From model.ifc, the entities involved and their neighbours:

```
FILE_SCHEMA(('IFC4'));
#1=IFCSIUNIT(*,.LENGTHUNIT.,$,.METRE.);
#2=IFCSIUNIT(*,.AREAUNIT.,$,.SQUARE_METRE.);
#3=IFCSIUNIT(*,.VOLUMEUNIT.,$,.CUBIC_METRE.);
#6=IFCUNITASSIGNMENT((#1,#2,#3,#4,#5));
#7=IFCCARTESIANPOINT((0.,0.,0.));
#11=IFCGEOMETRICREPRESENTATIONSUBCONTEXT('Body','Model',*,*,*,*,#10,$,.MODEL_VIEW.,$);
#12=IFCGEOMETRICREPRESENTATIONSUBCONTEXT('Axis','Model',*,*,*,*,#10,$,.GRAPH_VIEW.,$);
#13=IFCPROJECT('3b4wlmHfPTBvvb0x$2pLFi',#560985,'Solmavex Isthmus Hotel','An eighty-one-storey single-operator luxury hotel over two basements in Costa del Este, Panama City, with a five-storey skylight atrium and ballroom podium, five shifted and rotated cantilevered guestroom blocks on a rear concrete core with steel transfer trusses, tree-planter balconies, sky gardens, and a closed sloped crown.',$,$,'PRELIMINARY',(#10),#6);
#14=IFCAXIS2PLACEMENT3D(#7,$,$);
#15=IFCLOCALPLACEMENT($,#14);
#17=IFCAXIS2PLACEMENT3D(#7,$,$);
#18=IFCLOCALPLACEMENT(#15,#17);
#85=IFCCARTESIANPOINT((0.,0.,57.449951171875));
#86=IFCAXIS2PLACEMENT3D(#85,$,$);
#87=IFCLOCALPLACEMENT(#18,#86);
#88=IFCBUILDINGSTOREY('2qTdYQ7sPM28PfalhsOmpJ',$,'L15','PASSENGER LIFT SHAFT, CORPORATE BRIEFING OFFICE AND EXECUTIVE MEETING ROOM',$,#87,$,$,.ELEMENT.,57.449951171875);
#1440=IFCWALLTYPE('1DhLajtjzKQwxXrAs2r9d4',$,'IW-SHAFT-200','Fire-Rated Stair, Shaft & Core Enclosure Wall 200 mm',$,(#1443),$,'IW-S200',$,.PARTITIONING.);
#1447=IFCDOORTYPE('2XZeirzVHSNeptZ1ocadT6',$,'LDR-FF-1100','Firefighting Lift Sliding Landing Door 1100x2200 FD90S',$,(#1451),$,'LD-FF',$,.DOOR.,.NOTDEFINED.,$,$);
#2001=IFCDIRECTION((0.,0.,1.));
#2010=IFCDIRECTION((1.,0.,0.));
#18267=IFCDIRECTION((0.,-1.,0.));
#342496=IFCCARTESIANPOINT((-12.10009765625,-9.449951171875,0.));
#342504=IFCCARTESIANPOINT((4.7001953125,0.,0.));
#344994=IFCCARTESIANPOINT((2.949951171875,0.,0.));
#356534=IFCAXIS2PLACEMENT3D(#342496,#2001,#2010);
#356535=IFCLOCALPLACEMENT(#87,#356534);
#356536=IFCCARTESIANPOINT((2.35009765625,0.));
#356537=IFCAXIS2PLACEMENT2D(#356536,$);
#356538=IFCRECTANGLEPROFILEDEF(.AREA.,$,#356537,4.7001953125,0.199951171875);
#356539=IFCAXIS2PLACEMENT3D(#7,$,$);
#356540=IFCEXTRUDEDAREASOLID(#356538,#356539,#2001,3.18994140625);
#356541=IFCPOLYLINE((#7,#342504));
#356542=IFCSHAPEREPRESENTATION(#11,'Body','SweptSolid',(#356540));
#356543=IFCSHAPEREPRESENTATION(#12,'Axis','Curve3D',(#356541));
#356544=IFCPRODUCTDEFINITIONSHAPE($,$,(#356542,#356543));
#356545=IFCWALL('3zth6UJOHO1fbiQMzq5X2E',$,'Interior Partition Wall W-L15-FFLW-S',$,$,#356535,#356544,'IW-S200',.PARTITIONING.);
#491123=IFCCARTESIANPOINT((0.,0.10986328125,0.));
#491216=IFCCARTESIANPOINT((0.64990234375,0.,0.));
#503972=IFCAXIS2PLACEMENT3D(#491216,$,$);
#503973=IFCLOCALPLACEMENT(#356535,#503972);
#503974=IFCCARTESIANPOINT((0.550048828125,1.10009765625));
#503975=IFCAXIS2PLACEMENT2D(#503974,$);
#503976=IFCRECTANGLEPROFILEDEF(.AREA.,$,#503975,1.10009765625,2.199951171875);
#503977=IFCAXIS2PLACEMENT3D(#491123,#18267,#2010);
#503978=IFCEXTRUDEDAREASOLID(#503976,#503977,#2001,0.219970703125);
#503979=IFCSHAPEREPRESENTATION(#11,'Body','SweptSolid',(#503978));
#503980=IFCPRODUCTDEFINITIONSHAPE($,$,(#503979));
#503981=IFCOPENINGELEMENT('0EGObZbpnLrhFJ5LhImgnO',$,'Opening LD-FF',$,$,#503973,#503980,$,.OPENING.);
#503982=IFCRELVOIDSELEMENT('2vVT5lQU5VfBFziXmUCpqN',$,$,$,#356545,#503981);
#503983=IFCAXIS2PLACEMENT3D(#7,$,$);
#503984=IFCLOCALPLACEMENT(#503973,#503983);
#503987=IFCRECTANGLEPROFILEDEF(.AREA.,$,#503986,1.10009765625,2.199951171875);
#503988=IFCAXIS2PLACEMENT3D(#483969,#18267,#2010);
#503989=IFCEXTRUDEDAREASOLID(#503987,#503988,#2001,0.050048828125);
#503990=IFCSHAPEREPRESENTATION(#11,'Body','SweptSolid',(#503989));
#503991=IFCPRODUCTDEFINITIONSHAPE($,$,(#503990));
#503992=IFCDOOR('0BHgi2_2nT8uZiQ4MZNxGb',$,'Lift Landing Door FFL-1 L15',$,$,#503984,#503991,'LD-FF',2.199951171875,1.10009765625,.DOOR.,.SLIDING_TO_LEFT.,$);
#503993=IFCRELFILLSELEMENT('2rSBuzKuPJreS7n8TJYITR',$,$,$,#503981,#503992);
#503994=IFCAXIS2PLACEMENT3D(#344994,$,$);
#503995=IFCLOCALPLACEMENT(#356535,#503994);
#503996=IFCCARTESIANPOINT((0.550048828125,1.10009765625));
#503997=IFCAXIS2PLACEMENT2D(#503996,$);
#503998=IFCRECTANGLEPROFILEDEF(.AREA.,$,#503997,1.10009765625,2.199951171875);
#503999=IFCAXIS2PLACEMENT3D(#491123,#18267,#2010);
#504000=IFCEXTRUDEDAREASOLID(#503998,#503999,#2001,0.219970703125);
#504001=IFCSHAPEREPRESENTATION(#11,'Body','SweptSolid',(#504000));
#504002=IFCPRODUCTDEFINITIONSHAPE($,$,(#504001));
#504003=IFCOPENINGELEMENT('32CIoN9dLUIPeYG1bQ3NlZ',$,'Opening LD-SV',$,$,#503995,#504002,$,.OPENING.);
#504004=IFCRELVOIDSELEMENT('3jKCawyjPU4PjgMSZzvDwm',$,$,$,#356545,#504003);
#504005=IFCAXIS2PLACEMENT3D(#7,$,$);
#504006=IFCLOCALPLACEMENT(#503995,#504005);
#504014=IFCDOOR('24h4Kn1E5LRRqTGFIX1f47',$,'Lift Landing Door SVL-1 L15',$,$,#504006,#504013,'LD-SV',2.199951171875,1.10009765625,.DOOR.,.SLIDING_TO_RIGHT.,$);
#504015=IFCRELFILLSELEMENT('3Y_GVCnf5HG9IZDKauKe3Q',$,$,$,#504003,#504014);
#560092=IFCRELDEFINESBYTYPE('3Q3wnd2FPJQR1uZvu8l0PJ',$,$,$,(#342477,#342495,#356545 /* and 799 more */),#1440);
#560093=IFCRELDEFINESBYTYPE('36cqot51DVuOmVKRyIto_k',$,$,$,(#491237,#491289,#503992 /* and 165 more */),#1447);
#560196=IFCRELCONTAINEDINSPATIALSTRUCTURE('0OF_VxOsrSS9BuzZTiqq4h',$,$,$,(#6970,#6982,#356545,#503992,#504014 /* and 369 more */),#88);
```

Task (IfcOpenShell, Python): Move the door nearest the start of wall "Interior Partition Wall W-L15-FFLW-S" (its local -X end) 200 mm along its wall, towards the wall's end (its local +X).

```python
import ifcopenshell
import ifcopenshell.api.geometry
import ifcopenshell.util.placement

model = ifcopenshell.open("model.ifc")

door = model.by_id(503992)
opening = door.FillsVoids[0].RelatingOpeningElement
wall = opening.VoidsElements[0].RelatingBuildingElement

wall_matrix = ifcopenshell.util.placement.get_local_placement(wall.ObjectPlacement)
shift = wall_matrix[:3, 0] * 0.2
before = ifcopenshell.util.placement.get_local_placement(door.ObjectPlacement)[:3, 3].copy()

# The door is placed relative to its opening, so it follows when the opening moves.
matrix = ifcopenshell.util.placement.get_local_placement(opening.ObjectPlacement)
matrix[:3, 3] += shift
ifcopenshell.api.geometry.edit_object_placement(
    model, product=opening, matrix=matrix, is_si=False, should_transform_children=True
)

after = ifcopenshell.util.placement.get_local_placement(door.ObjectPlacement)[:3, 3]
print("door moved by", (after - before).round(3) + 0.0)

model.write("model_updated.ifc")
```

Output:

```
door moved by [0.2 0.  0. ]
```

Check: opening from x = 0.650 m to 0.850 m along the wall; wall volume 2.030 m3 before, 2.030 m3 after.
